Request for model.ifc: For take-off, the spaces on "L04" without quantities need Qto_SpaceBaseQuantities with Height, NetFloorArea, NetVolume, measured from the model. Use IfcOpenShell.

First a look at what the model holds.

```python
import ifcopenshell
import ifcopenshell.util.element
import ifcopenshell.util.unit

model = ifcopenshell.open("model.ifc")
print(model.schema)
for unit_type in ("LENGTHUNIT", "AREAUNIT", "VOLUMEUNIT"):
    print(unit_type, ifcopenshell.util.unit.calculate_unit_scale(model, unit_type))
storey = next(s for s in model.by_type("IfcBuildingStorey") if s.Name == "L04")
spaces = [e for e in ifcopenshell.util.element.get_decomposition(storey) if e.is_a("IfcSpace")]
for e in sorted(spaces, key=lambda e: e.id()):
    print(e.id(), e.is_a(), e.Name, list(ifcopenshell.util.element.get_psets(e, qtos_only=True)), sep=" | ")
```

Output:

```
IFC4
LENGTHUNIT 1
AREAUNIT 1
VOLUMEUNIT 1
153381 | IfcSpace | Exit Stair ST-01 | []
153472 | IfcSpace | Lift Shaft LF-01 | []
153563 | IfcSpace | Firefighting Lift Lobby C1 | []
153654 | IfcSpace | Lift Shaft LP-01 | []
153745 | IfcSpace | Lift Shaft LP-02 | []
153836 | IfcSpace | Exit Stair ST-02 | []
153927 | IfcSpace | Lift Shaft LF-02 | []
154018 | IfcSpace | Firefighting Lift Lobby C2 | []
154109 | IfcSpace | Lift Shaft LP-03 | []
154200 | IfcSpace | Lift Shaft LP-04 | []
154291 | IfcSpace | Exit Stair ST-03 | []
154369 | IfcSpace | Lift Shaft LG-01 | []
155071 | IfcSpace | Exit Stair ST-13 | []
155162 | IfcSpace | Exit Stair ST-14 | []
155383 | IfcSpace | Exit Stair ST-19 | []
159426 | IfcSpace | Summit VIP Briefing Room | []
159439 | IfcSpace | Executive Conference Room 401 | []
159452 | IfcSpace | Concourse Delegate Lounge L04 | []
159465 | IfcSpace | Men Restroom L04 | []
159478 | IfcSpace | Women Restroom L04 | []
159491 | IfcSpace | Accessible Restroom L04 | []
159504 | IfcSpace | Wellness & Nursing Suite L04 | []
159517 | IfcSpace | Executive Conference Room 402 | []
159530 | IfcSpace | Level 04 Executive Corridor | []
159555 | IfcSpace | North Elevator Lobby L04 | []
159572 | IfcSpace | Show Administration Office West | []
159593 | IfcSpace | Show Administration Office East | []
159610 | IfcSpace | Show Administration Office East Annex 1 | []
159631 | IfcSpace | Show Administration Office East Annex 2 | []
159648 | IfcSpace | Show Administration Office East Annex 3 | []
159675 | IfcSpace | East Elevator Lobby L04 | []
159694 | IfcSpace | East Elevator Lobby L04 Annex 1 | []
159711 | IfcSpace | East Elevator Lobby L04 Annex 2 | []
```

```python
import ifcopenshell
import ifcopenshell.api.pset
import ifcopenshell.geom
import ifcopenshell.util.element
import ifcopenshell.util.shape
import ifcopenshell.util.unit

model = ifcopenshell.open("model.ifc")
unit_scale = ifcopenshell.util.unit.calculate_unit_scale(model)
area_scale = ifcopenshell.util.unit.calculate_unit_scale(model, "AREAUNIT")
volume_scale = ifcopenshell.util.unit.calculate_unit_scale(model, "VOLUMEUNIT")
settings = ifcopenshell.geom.settings()

storey = next(s for s in model.by_type("IfcBuildingStorey") if s.Name == "L04")
spaces = [e for e in ifcopenshell.util.element.get_decomposition(storey) if e.is_a("IfcSpace")]

for e in sorted(spaces, key=lambda e: e.id()):
    if ifcopenshell.util.element.get_psets(e, qtos_only=True, should_inherit=False):
        continue
    # Geometry comes back in metres, in the element's own axes.
    shape = ifcopenshell.geom.create_shape(settings, e)
    values = {
        "Height": ifcopenshell.util.shape.get_z(shape.geometry) / unit_scale,
        "NetFloorArea": ifcopenshell.util.shape.get_footprint_area(shape.geometry) / area_scale,
        "NetVolume": ifcopenshell.util.shape.get_volume(shape.geometry) / volume_scale,
    }
    qto = ifcopenshell.api.pset.add_qto(model, product=e, name="Qto_SpaceBaseQuantities")
    ifcopenshell.api.pset.edit_qto(model, qto=qto, properties=values)
    print(e.id(), {k: round(v, 3) for k, v in values.items()})

model.write("model_rev.ifc")
```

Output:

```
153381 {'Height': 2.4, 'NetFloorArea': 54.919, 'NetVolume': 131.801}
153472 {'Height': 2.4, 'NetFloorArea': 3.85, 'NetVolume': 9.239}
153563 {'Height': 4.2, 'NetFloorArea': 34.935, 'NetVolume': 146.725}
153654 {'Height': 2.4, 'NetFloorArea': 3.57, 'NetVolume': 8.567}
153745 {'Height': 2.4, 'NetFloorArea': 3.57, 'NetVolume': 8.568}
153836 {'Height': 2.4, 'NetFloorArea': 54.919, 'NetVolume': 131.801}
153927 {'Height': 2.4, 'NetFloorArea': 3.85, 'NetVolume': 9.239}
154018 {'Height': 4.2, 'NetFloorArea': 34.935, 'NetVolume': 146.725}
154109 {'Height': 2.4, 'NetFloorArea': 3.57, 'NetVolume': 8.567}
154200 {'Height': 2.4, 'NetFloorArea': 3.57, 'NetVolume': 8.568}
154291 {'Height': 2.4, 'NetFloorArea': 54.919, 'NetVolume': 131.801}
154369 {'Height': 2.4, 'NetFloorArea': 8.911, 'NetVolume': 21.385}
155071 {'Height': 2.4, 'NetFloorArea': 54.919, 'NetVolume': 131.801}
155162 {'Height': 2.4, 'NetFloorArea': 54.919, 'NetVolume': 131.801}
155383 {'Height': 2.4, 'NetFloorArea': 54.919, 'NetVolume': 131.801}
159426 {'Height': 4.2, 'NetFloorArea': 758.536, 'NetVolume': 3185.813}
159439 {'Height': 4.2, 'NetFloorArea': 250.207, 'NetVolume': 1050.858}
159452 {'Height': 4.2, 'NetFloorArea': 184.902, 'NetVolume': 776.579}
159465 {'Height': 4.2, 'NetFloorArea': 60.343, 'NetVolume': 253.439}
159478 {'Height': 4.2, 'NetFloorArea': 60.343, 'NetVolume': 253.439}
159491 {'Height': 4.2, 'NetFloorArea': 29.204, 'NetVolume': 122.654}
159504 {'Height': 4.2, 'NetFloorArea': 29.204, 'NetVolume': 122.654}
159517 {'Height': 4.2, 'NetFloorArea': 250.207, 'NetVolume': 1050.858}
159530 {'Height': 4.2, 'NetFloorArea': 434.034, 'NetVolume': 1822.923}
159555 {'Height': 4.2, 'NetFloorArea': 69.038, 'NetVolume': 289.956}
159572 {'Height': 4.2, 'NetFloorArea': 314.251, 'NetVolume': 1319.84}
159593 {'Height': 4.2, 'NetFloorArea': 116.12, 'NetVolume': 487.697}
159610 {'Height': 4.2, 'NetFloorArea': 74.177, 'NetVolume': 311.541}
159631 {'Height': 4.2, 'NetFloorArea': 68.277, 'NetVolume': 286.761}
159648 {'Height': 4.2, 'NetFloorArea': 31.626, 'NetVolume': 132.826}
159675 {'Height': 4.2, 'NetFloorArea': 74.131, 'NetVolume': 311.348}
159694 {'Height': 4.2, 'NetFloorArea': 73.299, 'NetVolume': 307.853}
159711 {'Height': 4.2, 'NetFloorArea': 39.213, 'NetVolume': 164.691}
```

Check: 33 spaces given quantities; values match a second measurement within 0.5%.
